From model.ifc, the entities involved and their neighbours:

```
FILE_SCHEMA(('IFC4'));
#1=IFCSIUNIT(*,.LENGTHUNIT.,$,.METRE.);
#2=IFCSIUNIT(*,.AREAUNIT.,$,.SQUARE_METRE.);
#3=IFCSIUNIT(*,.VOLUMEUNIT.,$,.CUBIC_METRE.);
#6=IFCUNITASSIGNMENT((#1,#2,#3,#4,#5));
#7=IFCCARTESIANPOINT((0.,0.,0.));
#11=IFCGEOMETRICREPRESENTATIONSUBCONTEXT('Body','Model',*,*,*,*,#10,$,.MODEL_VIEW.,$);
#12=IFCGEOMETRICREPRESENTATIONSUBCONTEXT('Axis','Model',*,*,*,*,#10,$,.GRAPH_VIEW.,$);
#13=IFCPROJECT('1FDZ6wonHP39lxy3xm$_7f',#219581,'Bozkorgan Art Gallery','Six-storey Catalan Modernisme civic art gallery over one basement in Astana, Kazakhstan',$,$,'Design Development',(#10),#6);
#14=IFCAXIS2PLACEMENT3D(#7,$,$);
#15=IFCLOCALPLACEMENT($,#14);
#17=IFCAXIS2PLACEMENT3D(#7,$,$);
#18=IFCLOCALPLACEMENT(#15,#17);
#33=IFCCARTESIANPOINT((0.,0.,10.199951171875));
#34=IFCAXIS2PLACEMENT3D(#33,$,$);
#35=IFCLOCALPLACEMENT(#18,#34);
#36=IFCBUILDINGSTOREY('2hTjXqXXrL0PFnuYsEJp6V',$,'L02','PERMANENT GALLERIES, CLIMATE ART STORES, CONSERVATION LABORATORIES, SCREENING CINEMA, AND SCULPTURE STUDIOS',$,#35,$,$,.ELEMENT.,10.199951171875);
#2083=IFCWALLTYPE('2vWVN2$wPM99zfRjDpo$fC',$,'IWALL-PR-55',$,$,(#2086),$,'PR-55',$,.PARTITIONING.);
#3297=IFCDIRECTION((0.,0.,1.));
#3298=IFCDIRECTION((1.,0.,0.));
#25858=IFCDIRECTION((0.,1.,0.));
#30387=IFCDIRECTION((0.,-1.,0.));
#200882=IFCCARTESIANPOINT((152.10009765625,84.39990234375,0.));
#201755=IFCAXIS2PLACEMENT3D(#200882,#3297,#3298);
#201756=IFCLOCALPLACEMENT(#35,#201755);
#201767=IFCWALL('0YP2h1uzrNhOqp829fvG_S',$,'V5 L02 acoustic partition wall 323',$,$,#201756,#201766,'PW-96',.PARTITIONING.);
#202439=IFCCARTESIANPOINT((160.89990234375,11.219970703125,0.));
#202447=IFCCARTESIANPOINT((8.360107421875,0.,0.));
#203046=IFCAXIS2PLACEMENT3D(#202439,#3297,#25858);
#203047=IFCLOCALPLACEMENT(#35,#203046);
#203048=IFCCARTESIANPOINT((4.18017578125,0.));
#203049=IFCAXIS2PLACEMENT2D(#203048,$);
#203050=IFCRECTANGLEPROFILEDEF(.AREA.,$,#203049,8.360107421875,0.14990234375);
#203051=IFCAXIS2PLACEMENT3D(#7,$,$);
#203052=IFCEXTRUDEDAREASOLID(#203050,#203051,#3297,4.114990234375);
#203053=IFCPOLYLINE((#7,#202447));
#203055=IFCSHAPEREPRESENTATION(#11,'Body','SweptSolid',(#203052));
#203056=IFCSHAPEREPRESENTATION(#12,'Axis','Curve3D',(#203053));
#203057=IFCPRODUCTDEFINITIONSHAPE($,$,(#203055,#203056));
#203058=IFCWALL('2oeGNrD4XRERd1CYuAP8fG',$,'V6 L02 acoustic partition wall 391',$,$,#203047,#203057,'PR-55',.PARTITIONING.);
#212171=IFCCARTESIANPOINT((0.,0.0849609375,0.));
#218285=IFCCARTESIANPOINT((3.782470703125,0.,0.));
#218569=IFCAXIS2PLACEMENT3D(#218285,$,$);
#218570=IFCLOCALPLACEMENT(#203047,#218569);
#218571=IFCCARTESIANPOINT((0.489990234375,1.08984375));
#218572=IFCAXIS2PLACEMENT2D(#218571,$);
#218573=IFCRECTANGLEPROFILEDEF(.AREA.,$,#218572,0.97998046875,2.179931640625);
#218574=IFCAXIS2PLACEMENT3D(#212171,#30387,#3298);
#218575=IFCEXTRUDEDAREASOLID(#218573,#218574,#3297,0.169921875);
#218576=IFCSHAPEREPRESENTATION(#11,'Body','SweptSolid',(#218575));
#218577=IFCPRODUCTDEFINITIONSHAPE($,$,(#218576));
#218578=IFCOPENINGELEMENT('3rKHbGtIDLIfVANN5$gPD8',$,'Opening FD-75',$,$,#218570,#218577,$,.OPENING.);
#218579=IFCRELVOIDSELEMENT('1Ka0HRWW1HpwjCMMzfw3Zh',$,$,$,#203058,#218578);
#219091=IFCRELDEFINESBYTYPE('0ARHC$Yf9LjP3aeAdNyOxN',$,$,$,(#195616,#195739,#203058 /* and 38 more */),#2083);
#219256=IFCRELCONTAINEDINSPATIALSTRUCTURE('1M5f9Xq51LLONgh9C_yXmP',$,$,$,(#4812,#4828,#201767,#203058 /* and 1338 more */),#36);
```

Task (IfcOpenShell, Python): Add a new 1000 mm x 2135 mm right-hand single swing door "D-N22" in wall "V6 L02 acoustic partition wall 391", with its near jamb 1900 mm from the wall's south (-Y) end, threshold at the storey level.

```python
import numpy as np
import ifcopenshell
import ifcopenshell.api.feature
import ifcopenshell.api.geometry
import ifcopenshell.api.root
import ifcopenshell.api.spatial
import ifcopenshell.geom
import ifcopenshell.util.element
import ifcopenshell.util.placement
import ifcopenshell.util.representation
import ifcopenshell.util.shape
import ifcopenshell.util.unit

model = ifcopenshell.open("model.ifc")
unit_scale = ifcopenshell.util.unit.calculate_unit_scale(model)
settings = ifcopenshell.geom.settings()


def volume(element):
    """Net volume in cubic metres, openings subtracted."""
    shape = ifcopenshell.geom.create_shape(settings, element)
    return ifcopenshell.util.shape.get_volume(shape.geometry)


wall = model.by_id(203058)
storey = ifcopenshell.util.element.get_container(wall, ifc_class="IfcBuildingStorey")
context = ifcopenshell.util.representation.get_context(model, "Model", "Body", "MODEL_VIEW")
before = volume(wall)

width, height, from_end, sill = 1, 2.135, 1.9, 0.0  # metres

# The wall runs along its own X axis, and the end named is its -X end.
wall_shape = ifcopenshell.geom.create_shape(settings, wall)
x, y, z = ifcopenshell.util.shape.get_vertices(wall_shape.geometry).T
start = x.min() + from_end
face, thickness = float(y.min()), float(y.max() - y.min())
wall_matrix = ifcopenshell.util.placement.get_local_placement(wall.ObjectPlacement)
level = ifcopenshell.util.placement.get_local_placement(storey.ObjectPlacement)[2, 3]


def in_wall(x, y):
    """Placement at x, y metres in the wall's axes, at sill height."""
    matrix = wall_matrix.copy()
    matrix[:, 3] = wall_matrix @ np.array([x / unit_scale, y / unit_scale, 0.0, 1.0])
    matrix[2, 3] = level + sill / unit_scale
    return matrix


# Opening: a box that overshoots both wall faces by 50 mm.
opening = ifcopenshell.api.root.create_entity(model, ifc_class="IfcOpeningElement", predefined_type="OPENING")
box = ifcopenshell.api.geometry.add_wall_representation(
    model, context=context, length=width, height=height, thickness=thickness + 0.1
)
ifcopenshell.api.geometry.assign_representation(model, product=opening, representation=box)
ifcopenshell.api.geometry.edit_object_placement(model, product=opening, matrix=in_wall(start, face - 0.05), is_si=False)
ifcopenshell.api.feature.add_feature(model, feature=opening, element=wall)

door = ifcopenshell.api.root.create_entity(model, ifc_class="IfcDoor", name="D-N22", predefined_type="DOOR")
door.OverallWidth, door.OverallHeight = width / unit_scale, height / unit_scale
door.OperationType = "SINGLE_SWING_RIGHT"
body = ifcopenshell.api.geometry.add_door_representation(
    model,
    context=context,
    overall_width=door.OverallWidth,
    overall_height=door.OverallHeight,
    operation_type="SINGLE_SWING_RIGHT",
    lining_properties={"LiningDepth": thickness / unit_scale, "ThresholdDepth": thickness / unit_scale},
)
ifcopenshell.api.geometry.assign_representation(model, product=door, representation=body)
ifcopenshell.api.spatial.assign_container(model, products=[door], relating_structure=storey)
ifcopenshell.api.feature.add_filling(model, opening=opening, element=door)

# The lining spans the wall, so the door starts at the wall face.
ifcopenshell.api.geometry.edit_object_placement(model, product=door, matrix=in_wall(start, face), is_si=False)

after = volume(wall)

print(f"wall volume {before:.3f} -> {after:.3f} m3")

model.write("model_v2.ifc")
```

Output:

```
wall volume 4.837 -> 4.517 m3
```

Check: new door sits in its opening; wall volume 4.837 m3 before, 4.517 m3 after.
